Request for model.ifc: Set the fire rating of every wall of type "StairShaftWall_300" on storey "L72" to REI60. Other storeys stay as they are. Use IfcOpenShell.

First a look at what the model holds.

```python
import ifcopenshell
import ifcopenshell.util.element

model = ifcopenshell.open("model.ifc")
print(model.schema)
storey = next(s for s in model.by_type("IfcBuildingStorey") if s.Name == "L72")
walls = [e for e in ifcopenshell.util.element.get_decomposition(storey) if e.is_a("IfcWall")]
seen = {}
for e in walls:
    element_type = ifcopenshell.util.element.get_type(e)
    key = (element_type.Name if element_type != e and element_type else None, ifcopenshell.util.element.get_pset(e, "Pset_WallCommon", "FireRating"))
    seen[key] = seen.get(key, 0) + 1
for (name, value), count in sorted(seen.items(), key=str):
    print(count, "x", name, "|", value)
```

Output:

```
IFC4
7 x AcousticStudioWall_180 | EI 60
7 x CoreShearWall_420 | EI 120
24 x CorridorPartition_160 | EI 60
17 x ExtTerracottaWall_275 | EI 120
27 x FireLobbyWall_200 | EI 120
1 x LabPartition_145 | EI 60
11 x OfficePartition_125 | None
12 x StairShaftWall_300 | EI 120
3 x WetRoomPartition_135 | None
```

```python
import ifcopenshell
import ifcopenshell.api.pset
import ifcopenshell.util.element

model = ifcopenshell.open("model.ifc")

storey = next(s for s in model.by_type("IfcBuildingStorey") if s.Name == "L72")
walls = [e for e in ifcopenshell.util.element.get_decomposition(storey) if e.is_a("IfcWall")]

count = 0
for e in walls:
    element_type = ifcopenshell.util.element.get_type(e)
    if element_type in (None, e) or element_type.Name != "StairShaftWall_300":
        continue
    # add_pset returns the element's existing set when there is one.
    pset = ifcopenshell.api.pset.add_pset(model, product=e, name="Pset_WallCommon")
    ifcopenshell.api.pset.edit_pset(model, pset=pset, properties={"FireRating": "REI60"})
    count += 1

print(count, "walls updated")

model.write("model_rev.ifc")
```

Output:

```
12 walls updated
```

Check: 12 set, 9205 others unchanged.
